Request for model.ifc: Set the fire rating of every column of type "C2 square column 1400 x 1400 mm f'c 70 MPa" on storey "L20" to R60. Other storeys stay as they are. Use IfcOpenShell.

First a look at what the model holds.

```python
import ifcopenshell
import ifcopenshell.util.element

model = ifcopenshell.open("model.ifc")
print(model.schema)
storey = next(s for s in model.by_type("IfcBuildingStorey") if s.Name == "L20")
columns = [e for e in ifcopenshell.util.element.get_decomposition(storey) if e.is_a("IfcColumn")]
seen = {}
for e in columns:
    element_type = ifcopenshell.util.element.get_type(e)
    key = (element_type.Name if element_type != e and element_type else None, ifcopenshell.util.element.get_pset(e, "Pset_ColumnCommon", "FireRating"))
    seen[key] = seen.get(key, 0) + 1
for (name, value), count in sorted(seen.items(), key=str):
    print(count, "x", name, "|", value)
```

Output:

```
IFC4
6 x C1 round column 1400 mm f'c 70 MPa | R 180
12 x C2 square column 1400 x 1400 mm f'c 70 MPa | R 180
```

```python
import ifcopenshell
import ifcopenshell.api.pset
import ifcopenshell.util.element

model = ifcopenshell.open("model.ifc")

storey = next(s for s in model.by_type("IfcBuildingStorey") if s.Name == "L20")
columns = [e for e in ifcopenshell.util.element.get_decomposition(storey) if e.is_a("IfcColumn")]

count = 0
for e in columns:
    element_type = ifcopenshell.util.element.get_type(e)
    if element_type in (None, e) or element_type.Name != "C2 square column 1400 x 1400 mm f'c 70 MPa":
        continue
    found = ifcopenshell.util.element.get_pset(e, "Pset_ColumnCommon", should_inherit=False)
    if found:
        pset = model.by_id(found["id"])
        if len(ifcopenshell.util.element.get_elements_by_pset(pset)) > 1:
            pset = ifcopenshell.api.pset.unshare_pset(model, products=[e], pset=pset)[0]
    else:
        pset = ifcopenshell.api.pset.add_pset(model, product=e, name="Pset_ColumnCommon")
    ifcopenshell.api.pset.edit_pset(model, pset=pset, properties={"FireRating": "R60"})
    count += 1

print(count, "columns updated")

model.write("model_v2.ifc")
```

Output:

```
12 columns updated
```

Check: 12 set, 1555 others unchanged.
